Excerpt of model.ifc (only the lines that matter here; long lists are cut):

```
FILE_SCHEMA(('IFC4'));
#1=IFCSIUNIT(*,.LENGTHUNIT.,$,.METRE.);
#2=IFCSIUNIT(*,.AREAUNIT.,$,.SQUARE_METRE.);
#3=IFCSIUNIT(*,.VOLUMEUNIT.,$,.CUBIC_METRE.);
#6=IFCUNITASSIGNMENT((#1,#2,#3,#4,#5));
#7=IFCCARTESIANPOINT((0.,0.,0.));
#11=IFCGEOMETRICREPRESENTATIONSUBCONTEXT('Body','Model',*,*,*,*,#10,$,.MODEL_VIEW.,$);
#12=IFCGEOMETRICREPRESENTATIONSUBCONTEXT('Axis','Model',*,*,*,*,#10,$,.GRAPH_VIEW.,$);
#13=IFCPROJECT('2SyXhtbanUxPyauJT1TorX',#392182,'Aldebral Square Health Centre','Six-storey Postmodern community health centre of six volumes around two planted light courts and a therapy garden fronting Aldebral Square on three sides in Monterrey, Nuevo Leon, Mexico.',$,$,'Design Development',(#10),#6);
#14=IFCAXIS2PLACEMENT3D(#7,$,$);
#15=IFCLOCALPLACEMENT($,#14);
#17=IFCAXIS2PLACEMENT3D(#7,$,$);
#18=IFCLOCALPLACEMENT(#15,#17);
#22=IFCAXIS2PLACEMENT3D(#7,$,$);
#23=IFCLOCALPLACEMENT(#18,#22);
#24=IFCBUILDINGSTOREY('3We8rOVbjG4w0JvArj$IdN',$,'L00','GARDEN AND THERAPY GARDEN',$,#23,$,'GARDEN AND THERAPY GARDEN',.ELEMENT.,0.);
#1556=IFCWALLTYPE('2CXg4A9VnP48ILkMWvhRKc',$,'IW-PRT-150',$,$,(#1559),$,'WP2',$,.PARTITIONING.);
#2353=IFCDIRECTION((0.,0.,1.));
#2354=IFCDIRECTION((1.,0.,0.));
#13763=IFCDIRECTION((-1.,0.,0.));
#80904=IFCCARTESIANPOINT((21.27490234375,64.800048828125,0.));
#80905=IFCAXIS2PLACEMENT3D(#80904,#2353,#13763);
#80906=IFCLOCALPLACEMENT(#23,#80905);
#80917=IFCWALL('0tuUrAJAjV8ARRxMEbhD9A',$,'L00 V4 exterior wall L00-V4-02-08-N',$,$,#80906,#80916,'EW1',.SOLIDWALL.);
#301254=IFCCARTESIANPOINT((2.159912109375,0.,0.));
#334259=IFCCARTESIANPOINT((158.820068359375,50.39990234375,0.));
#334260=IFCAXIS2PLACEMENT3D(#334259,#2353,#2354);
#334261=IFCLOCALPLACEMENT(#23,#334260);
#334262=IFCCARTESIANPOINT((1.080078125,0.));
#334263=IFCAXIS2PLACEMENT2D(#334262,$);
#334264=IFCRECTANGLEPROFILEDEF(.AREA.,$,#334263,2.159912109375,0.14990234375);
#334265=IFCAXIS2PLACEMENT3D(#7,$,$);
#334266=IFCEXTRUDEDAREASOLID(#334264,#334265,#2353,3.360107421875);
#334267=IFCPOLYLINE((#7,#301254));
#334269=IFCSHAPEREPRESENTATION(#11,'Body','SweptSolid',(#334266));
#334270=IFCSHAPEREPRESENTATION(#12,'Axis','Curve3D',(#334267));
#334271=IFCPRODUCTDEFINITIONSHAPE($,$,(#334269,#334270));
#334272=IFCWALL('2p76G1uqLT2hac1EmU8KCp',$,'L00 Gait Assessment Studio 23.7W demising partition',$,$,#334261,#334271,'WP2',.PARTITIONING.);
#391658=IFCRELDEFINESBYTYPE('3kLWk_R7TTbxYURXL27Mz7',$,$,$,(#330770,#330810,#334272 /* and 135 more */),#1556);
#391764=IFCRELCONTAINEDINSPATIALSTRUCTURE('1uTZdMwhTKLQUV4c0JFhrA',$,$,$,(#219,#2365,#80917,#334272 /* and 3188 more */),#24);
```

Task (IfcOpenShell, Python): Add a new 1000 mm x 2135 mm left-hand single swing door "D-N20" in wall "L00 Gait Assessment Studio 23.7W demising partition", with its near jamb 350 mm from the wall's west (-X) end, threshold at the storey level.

```python
import numpy as np
import ifcopenshell
import ifcopenshell.api.feature
import ifcopenshell.api.geometry
import ifcopenshell.api.root
import ifcopenshell.api.spatial
import ifcopenshell.geom
import ifcopenshell.util.element
import ifcopenshell.util.placement
import ifcopenshell.util.representation
import ifcopenshell.util.shape
import ifcopenshell.util.unit

model = ifcopenshell.open("model.ifc")
unit_scale = ifcopenshell.util.unit.calculate_unit_scale(model)
settings = ifcopenshell.geom.settings()


def volume(element):
    """Net volume in cubic metres, openings subtracted."""
    shape = ifcopenshell.geom.create_shape(settings, element)
    return ifcopenshell.util.shape.get_volume(shape.geometry)


wall = model.by_guid("2p76G1uqLT2hac1EmU8KCp")
storey = ifcopenshell.util.element.get_container(wall, ifc_class="IfcBuildingStorey")
context = ifcopenshell.util.representation.get_context(model, "Model", "Body", "MODEL_VIEW")
before = volume(wall)

width, height, from_end, sill = 1, 2.135, 0.35, 0.0  # metres

# The wall runs along its own X axis, and the end named is its -X end.
wall_shape = ifcopenshell.geom.create_shape(settings, wall)
x, y, z = ifcopenshell.util.shape.get_vertices(wall_shape.geometry).T
start = x.min() + from_end
face, thickness = float(y.min()), float(y.max() - y.min())
wall_matrix = ifcopenshell.util.placement.get_local_placement(wall.ObjectPlacement)
level = ifcopenshell.util.placement.get_local_placement(storey.ObjectPlacement)[2, 3]


def in_wall(x, y):
    """Placement at x, y metres in the wall's axes, at sill height."""
    matrix = wall_matrix.copy()
    matrix[:, 3] = wall_matrix @ np.array([x / unit_scale, y / unit_scale, 0.0, 1.0])
    matrix[2, 3] = level + sill / unit_scale
    return matrix


# Opening: a box that overshoots both wall faces by 50 mm.
opening = ifcopenshell.api.root.create_entity(model, ifc_class="IfcOpeningElement", predefined_type="OPENING")
box = ifcopenshell.api.geometry.add_wall_representation(
    model, context=context, length=width, height=height, thickness=thickness + 0.1
)
ifcopenshell.api.geometry.assign_representation(model, product=opening, representation=box)
ifcopenshell.api.geometry.edit_object_placement(model, product=opening, matrix=in_wall(start, face - 0.05), is_si=False)
ifcopenshell.api.feature.add_feature(model, feature=opening, element=wall)

door = ifcopenshell.api.root.create_entity(model, ifc_class="IfcDoor", name="D-N20", predefined_type="DOOR")
door.OverallWidth, door.OverallHeight = width / unit_scale, height / unit_scale
door.OperationType = "SINGLE_SWING_LEFT"
body = ifcopenshell.api.geometry.add_door_representation(
    model,
    context=context,
    overall_width=door.OverallWidth,
    overall_height=door.OverallHeight,
    operation_type="SINGLE_SWING_LEFT",
    lining_properties={"LiningDepth": thickness / unit_scale, "ThresholdDepth": thickness / unit_scale},
)
ifcopenshell.api.geometry.assign_representation(model, product=door, representation=body)
ifcopenshell.api.spatial.assign_container(model, products=[door], relating_structure=storey)
ifcopenshell.api.feature.add_filling(model, opening=opening, element=door)

# The lining spans the wall, so the door starts at the wall face.
ifcopenshell.api.geometry.edit_object_placement(model, product=door, matrix=in_wall(start, face), is_si=False)

after = volume(wall)

print(f"wall volume {before:.3f} -> {after:.3f} m3")

model.write("model_v2.ifc")
```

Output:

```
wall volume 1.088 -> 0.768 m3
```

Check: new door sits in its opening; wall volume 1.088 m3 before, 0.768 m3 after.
